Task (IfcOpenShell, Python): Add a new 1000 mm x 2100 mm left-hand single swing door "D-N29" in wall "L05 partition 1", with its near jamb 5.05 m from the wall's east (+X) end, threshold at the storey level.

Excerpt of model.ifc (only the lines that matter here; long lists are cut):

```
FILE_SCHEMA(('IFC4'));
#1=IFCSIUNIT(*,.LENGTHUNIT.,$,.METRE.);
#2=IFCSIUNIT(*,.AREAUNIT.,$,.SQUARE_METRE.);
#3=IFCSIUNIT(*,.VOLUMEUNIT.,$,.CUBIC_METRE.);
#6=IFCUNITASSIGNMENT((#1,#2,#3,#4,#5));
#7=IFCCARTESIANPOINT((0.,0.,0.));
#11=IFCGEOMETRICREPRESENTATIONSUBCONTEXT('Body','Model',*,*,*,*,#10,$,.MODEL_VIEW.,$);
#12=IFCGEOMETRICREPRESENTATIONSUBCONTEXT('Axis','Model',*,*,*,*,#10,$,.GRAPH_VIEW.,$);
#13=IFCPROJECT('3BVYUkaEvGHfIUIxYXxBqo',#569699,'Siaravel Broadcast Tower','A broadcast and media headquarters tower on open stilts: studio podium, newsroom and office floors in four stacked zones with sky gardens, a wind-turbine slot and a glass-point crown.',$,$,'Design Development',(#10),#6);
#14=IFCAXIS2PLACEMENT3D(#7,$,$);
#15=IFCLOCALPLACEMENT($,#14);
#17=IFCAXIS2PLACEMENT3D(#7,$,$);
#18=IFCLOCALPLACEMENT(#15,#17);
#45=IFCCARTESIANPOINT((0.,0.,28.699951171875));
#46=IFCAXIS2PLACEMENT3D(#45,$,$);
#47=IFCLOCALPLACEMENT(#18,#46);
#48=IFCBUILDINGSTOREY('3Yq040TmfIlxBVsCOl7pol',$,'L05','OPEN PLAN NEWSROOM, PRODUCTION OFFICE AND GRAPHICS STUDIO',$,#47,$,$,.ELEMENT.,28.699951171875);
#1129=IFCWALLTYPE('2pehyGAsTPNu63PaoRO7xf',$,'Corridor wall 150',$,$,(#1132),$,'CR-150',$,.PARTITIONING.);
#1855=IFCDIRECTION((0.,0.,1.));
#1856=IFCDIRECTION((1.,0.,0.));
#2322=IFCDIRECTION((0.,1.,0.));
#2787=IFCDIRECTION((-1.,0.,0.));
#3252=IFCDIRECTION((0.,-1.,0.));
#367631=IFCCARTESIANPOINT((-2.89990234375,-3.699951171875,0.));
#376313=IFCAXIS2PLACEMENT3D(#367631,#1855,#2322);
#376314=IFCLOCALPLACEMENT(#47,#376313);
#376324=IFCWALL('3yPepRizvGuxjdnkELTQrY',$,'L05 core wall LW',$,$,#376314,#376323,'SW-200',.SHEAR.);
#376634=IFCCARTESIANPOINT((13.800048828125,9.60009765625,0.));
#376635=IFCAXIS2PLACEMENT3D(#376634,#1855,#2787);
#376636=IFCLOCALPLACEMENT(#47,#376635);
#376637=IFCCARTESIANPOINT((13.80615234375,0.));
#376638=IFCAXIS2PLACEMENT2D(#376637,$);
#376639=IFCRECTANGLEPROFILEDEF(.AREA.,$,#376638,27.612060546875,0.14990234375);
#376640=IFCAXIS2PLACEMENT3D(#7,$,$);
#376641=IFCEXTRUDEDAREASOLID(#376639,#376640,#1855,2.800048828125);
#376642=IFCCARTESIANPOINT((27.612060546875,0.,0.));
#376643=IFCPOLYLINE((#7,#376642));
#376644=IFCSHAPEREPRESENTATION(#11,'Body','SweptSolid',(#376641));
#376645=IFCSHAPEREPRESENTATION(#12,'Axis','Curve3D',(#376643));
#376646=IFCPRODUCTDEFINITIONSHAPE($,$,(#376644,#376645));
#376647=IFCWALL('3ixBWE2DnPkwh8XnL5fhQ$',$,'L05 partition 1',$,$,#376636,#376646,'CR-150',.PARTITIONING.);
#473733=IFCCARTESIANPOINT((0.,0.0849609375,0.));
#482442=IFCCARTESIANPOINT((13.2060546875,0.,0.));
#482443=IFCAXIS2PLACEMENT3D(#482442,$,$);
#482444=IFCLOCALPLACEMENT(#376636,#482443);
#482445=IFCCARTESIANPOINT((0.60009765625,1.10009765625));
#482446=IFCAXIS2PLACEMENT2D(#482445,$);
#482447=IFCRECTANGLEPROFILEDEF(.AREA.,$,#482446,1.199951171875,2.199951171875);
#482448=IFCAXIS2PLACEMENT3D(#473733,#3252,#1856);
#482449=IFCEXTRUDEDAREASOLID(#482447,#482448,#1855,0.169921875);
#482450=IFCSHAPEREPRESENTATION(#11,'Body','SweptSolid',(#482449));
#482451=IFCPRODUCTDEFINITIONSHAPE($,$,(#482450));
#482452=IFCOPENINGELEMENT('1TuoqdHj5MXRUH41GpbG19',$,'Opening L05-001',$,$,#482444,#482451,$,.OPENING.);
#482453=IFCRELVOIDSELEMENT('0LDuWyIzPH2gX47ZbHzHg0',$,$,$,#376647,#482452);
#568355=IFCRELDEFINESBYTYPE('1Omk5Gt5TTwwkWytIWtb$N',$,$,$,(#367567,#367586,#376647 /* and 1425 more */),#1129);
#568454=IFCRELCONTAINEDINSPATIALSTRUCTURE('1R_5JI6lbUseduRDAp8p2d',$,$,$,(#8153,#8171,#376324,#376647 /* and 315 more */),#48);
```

```python
import numpy as np
import ifcopenshell
import ifcopenshell.api.feature
import ifcopenshell.api.geometry
import ifcopenshell.api.root
import ifcopenshell.api.spatial
import ifcopenshell.geom
import ifcopenshell.util.element
import ifcopenshell.util.placement
import ifcopenshell.util.representation
import ifcopenshell.util.shape
import ifcopenshell.util.unit

model = ifcopenshell.open("model.ifc")
unit_scale = ifcopenshell.util.unit.calculate_unit_scale(model)
settings = ifcopenshell.geom.settings()


def volume(element):
    """Net volume in cubic metres, openings subtracted."""
    shape = ifcopenshell.geom.create_shape(settings, element)
    return ifcopenshell.util.shape.get_volume(shape.geometry)


wall = model.by_guid("3ixBWE2DnPkwh8XnL5fhQ$")
storey = ifcopenshell.util.element.get_container(wall, ifc_class="IfcBuildingStorey")
context = ifcopenshell.util.representation.get_context(model, "Model", "Body", "MODEL_VIEW")
before = volume(wall)

width, height, from_end, sill = 1, 2.1, 5.05, 0.0  # metres

# The wall runs along its own X axis, and the end named is its -X end.
wall_shape = ifcopenshell.geom.create_shape(settings, wall)
x, y, z = ifcopenshell.util.shape.get_vertices(wall_shape.geometry).T
start = x.min() + from_end
face, thickness = float(y.min()), float(y.max() - y.min())
wall_matrix = ifcopenshell.util.placement.get_local_placement(wall.ObjectPlacement)
level = ifcopenshell.util.placement.get_local_placement(storey.ObjectPlacement)[2, 3]


def in_wall(x, y):
    """Placement at x, y metres in the wall's axes, at sill height."""
    matrix = wall_matrix.copy()
    matrix[:, 3] = wall_matrix @ np.array([x / unit_scale, y / unit_scale, 0.0, 1.0])
    matrix[2, 3] = level + sill / unit_scale
    return matrix


# Opening: a box that overshoots both wall faces by 50 mm.
opening = ifcopenshell.api.root.create_entity(model, ifc_class="IfcOpeningElement", predefined_type="OPENING")
box = ifcopenshell.api.geometry.add_wall_representation(
    model, context=context, length=width, height=height, thickness=thickness + 0.1
)
ifcopenshell.api.geometry.assign_representation(model, product=opening, representation=box)
ifcopenshell.api.geometry.edit_object_placement(model, product=opening, matrix=in_wall(start, face - 0.05), is_si=False)
ifcopenshell.api.feature.add_feature(model, feature=opening, element=wall)

door = ifcopenshell.api.root.create_entity(model, ifc_class="IfcDoor", name="D-N29", predefined_type="DOOR")
door.OverallWidth, door.OverallHeight = width / unit_scale, height / unit_scale
door.OperationType = "SINGLE_SWING_LEFT"
body = ifcopenshell.api.geometry.add_door_representation(
    model,
    context=context,
    overall_width=door.OverallWidth,
    overall_height=door.OverallHeight,
    operation_type="SINGLE_SWING_LEFT",
    lining_properties={"LiningDepth": thickness / unit_scale, "ThresholdDepth": thickness / unit_scale},
)
ifcopenshell.api.geometry.assign_representation(model, product=door, representation=body)
ifcopenshell.api.spatial.assign_container(model, products=[door], relating_structure=storey)
ifcopenshell.api.feature.add_filling(model, opening=opening, element=door)

# The lining spans the wall, so the door starts at the wall face.
ifcopenshell.api.geometry.edit_object_placement(model, product=door, matrix=in_wall(start, face), is_si=False)

after = volume(wall)

print(f"wall volume {before:.3f} -> {after:.3f} m3")

model.write("model-out.ifc")
```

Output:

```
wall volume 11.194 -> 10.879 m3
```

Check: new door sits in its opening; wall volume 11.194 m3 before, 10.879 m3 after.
